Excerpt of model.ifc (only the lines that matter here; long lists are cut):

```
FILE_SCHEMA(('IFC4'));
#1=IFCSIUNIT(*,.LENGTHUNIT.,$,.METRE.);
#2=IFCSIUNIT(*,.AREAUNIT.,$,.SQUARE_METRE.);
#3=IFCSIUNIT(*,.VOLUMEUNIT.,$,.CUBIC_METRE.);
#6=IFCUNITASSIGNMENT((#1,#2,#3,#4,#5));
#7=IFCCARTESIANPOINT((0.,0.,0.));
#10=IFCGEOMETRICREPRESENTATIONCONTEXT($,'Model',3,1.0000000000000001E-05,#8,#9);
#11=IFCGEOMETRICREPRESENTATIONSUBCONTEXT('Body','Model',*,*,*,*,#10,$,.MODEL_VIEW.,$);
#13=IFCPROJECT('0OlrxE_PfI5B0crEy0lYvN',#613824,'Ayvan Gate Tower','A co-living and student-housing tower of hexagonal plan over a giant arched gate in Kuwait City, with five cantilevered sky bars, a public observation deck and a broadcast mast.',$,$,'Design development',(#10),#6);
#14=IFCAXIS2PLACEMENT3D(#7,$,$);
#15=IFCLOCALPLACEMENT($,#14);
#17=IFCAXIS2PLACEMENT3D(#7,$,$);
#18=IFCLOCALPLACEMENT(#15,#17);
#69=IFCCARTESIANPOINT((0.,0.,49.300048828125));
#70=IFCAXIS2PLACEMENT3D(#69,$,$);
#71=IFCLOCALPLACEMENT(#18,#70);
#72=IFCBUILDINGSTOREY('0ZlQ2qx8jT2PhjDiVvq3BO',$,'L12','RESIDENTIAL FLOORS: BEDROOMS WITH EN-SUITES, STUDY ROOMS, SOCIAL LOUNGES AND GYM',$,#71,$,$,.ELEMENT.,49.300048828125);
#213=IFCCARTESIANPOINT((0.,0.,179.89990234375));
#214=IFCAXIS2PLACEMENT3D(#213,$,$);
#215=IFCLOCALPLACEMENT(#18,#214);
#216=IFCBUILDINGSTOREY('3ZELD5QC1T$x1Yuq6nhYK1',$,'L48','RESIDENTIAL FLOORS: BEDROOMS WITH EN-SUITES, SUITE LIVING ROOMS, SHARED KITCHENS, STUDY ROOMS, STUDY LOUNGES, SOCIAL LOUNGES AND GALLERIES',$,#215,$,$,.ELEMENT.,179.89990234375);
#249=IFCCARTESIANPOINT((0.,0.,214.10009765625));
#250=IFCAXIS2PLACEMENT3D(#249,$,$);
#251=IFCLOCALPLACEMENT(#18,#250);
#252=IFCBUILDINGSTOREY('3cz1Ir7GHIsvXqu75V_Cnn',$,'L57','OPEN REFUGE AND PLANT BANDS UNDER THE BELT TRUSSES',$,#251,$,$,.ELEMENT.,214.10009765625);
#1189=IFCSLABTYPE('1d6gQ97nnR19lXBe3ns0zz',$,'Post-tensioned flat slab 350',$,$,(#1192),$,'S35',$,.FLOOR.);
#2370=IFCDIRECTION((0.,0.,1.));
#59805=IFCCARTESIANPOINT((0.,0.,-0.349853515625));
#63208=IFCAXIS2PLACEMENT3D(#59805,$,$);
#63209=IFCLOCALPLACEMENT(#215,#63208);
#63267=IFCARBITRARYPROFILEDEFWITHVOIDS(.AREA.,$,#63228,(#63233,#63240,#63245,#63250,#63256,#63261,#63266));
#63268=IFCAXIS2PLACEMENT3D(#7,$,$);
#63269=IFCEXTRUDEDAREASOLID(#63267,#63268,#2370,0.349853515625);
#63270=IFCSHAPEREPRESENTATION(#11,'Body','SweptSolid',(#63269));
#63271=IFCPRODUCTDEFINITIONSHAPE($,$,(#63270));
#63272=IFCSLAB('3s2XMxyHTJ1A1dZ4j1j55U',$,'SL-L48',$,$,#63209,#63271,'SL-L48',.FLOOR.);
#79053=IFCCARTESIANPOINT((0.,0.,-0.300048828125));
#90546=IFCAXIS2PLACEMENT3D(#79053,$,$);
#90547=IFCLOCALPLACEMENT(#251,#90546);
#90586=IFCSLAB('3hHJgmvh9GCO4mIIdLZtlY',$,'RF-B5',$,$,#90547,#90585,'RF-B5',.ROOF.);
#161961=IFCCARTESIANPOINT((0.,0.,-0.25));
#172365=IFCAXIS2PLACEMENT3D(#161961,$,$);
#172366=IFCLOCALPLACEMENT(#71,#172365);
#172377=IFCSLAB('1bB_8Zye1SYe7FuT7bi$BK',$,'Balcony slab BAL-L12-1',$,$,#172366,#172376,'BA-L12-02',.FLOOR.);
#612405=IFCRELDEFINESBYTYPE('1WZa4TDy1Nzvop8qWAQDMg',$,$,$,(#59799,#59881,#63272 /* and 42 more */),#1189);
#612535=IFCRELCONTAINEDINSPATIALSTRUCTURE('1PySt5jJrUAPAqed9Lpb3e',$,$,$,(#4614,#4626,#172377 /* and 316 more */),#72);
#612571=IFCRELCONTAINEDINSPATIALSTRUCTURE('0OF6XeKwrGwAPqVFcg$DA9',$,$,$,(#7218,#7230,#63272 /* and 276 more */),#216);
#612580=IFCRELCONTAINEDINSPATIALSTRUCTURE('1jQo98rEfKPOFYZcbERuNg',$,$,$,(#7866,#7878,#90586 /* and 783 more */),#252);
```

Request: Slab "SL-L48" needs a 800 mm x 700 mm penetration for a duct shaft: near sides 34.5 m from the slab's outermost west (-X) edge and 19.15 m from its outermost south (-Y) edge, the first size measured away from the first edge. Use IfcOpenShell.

```python
import numpy as np
import ifcopenshell
import ifcopenshell.api.feature
import ifcopenshell.api.geometry
import ifcopenshell.api.root
import ifcopenshell.geom
import ifcopenshell.util.placement
import ifcopenshell.util.representation
import ifcopenshell.util.shape
import ifcopenshell.util.unit

model = ifcopenshell.open("model.ifc")
unit_scale = ifcopenshell.util.unit.calculate_unit_scale(model)
settings = ifcopenshell.geom.settings()


def volume(element):
    """Net volume in cubic metres, openings subtracted."""
    shape = ifcopenshell.geom.create_shape(settings, element)
    return ifcopenshell.util.shape.get_volume(shape.geometry)


slab = model.by_guid("3s2XMxyHTJ1A1dZ4j1j55U")
before = volume(slab)

# Extent in the slab's own axes, in metres. The edges named are its -X and -Y sides.
slab_shape = ifcopenshell.geom.create_shape(settings, slab)
vertices = ifcopenshell.util.shape.get_vertices(slab_shape.geometry)
x_min, y_min, bottom = vertices.min(axis=0)
top = vertices[:, 2].max()

opening = ifcopenshell.api.root.create_entity(model, ifc_class="IfcOpeningElement", name="Duct shaft opening", predefined_type="OPENING")
context = ifcopenshell.util.representation.get_context(model, "Model", "Body", "MODEL_VIEW")
width, depth = 0.8, 0.7
outline = [(0.0, 0.0), (width, 0.0), (width, depth), (0.0, depth), (0.0, 0.0)]
# Overshoot both faces by 50 mm so the cut is clean.
shape = ifcopenshell.api.geometry.add_slab_representation(
    model, context=context, depth=top - bottom + 0.1, polyline=outline
)
ifcopenshell.api.geometry.assign_representation(model, product=opening, representation=shape)

matrix = ifcopenshell.util.placement.get_local_placement(slab.ObjectPlacement)
matrix[:, 3] = matrix @ np.append(np.array([x_min + 34.5, y_min + 19.15, bottom - 0.05]) / unit_scale, 1.0)
ifcopenshell.api.geometry.edit_object_placement(model, product=opening, matrix=matrix, is_si=False)
ifcopenshell.api.feature.add_feature(model, feature=opening, element=slab)

after = volume(slab)

print(f"slab volume {before:.3f} -> {after:.3f} m3")

model.write("model_rev.ifc")
```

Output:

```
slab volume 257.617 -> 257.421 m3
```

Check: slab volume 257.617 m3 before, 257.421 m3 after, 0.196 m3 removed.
